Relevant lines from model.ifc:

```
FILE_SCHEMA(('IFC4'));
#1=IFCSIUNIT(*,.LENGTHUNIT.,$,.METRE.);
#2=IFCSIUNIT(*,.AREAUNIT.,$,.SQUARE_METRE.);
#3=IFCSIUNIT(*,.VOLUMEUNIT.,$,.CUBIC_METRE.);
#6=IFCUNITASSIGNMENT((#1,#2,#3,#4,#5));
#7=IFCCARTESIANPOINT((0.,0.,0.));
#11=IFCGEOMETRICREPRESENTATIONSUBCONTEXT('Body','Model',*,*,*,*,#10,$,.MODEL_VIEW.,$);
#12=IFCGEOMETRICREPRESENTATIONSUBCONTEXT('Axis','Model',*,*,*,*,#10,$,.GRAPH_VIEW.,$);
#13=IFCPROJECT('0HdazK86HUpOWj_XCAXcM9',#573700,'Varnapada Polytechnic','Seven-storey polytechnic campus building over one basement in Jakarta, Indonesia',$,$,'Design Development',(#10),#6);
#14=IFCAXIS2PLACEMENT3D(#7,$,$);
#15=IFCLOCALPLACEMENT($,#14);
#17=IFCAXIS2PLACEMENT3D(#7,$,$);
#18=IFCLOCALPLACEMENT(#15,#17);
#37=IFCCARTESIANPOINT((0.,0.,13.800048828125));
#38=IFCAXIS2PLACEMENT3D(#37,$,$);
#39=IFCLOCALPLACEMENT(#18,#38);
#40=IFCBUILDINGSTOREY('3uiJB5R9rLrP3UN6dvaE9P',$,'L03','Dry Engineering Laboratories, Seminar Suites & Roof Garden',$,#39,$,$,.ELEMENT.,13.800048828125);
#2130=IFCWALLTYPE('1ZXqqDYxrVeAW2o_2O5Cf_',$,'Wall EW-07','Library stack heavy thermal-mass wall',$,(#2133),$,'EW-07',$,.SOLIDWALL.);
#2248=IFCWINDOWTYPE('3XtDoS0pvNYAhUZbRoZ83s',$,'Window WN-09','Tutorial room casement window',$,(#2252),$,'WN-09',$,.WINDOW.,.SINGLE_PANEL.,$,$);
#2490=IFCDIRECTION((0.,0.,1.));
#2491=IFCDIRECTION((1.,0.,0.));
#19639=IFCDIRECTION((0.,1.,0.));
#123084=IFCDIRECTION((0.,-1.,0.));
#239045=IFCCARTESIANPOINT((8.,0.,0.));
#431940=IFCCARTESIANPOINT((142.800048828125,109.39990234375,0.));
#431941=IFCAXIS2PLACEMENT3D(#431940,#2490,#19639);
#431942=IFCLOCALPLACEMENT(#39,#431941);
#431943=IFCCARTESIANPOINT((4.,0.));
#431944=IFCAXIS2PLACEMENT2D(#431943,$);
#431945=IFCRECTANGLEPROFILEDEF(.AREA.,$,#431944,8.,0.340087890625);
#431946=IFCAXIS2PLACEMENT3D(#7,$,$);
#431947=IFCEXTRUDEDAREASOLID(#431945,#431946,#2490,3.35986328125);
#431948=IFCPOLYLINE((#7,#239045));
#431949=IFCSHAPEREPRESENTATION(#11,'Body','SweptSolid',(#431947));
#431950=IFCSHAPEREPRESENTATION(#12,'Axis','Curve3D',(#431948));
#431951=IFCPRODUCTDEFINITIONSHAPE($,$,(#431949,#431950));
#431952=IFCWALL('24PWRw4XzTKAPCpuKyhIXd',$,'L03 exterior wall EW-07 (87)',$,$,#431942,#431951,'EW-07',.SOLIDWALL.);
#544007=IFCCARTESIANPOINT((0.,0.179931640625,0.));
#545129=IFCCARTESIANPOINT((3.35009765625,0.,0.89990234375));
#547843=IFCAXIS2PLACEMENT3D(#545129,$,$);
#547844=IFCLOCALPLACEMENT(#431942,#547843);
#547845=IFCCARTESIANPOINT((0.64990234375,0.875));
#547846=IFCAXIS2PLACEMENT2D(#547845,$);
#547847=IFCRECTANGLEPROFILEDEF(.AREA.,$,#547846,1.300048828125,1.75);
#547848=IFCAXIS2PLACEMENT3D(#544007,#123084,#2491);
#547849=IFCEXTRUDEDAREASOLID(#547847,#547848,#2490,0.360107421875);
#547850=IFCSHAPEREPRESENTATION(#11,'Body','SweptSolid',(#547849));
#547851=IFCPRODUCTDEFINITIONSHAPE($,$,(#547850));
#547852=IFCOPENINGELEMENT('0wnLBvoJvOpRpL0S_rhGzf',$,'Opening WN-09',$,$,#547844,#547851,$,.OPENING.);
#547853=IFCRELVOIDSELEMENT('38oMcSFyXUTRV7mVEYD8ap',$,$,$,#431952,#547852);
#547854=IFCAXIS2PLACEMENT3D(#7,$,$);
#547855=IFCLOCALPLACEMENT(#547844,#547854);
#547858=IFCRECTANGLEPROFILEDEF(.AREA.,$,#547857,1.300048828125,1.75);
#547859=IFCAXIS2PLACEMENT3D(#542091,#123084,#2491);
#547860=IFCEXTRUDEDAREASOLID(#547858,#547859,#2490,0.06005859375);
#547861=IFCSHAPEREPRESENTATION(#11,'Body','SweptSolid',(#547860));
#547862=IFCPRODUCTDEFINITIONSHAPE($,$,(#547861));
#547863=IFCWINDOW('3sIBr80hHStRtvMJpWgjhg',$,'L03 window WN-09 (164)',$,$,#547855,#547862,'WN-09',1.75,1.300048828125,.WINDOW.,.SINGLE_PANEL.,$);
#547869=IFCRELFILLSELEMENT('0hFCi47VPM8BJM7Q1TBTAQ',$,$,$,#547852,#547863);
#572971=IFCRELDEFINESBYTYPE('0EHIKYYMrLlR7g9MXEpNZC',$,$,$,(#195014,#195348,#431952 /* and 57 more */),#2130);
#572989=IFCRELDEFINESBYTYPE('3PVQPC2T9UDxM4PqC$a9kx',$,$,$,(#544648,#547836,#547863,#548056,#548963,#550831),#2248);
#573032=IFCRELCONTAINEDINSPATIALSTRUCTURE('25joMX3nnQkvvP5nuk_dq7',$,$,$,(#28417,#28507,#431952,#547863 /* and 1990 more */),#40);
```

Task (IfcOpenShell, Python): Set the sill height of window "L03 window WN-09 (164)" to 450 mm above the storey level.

```python
import numpy as np
import ifcopenshell
import ifcopenshell.api.geometry
import ifcopenshell.geom
import ifcopenshell.util.element
import ifcopenshell.util.placement
import ifcopenshell.util.shape
import ifcopenshell.util.unit

model = ifcopenshell.open("model.ifc")
unit_scale = ifcopenshell.util.unit.calculate_unit_scale(model)

window = model.by_guid("3sIBr80hHStRtvMJpWgjhg")
opening = window.FillsVoids[0].RelatingOpeningElement
storey = ifcopenshell.util.element.get_container(window, ifc_class="IfcBuildingStorey")
level = ifcopenshell.util.placement.get_local_placement(storey.ObjectPlacement)[2, 3]

# The opening's origin need not be at the sill, so measure its lowest point.
shape = ifcopenshell.geom.create_shape(ifcopenshell.geom.settings(), opening)
bottom = ifcopenshell.util.shape.get_shape_bottom_elevation(shape, shape.geometry) / unit_scale
dz = level + 0.45 - bottom

shift = np.array([0.0, 0.0, dz])
# The window is placed relative to its opening, so it follows when the opening moves.
matrix = ifcopenshell.util.placement.get_local_placement(opening.ObjectPlacement)
matrix[:3, 3] += shift
ifcopenshell.api.geometry.edit_object_placement(
    model, product=opening, matrix=matrix, is_si=False, should_transform_children=True
)

print(f"moved by {dz * unit_scale:+.3f} m")

model.write("model_rev.ifc")
```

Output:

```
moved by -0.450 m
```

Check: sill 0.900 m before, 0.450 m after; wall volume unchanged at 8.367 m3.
